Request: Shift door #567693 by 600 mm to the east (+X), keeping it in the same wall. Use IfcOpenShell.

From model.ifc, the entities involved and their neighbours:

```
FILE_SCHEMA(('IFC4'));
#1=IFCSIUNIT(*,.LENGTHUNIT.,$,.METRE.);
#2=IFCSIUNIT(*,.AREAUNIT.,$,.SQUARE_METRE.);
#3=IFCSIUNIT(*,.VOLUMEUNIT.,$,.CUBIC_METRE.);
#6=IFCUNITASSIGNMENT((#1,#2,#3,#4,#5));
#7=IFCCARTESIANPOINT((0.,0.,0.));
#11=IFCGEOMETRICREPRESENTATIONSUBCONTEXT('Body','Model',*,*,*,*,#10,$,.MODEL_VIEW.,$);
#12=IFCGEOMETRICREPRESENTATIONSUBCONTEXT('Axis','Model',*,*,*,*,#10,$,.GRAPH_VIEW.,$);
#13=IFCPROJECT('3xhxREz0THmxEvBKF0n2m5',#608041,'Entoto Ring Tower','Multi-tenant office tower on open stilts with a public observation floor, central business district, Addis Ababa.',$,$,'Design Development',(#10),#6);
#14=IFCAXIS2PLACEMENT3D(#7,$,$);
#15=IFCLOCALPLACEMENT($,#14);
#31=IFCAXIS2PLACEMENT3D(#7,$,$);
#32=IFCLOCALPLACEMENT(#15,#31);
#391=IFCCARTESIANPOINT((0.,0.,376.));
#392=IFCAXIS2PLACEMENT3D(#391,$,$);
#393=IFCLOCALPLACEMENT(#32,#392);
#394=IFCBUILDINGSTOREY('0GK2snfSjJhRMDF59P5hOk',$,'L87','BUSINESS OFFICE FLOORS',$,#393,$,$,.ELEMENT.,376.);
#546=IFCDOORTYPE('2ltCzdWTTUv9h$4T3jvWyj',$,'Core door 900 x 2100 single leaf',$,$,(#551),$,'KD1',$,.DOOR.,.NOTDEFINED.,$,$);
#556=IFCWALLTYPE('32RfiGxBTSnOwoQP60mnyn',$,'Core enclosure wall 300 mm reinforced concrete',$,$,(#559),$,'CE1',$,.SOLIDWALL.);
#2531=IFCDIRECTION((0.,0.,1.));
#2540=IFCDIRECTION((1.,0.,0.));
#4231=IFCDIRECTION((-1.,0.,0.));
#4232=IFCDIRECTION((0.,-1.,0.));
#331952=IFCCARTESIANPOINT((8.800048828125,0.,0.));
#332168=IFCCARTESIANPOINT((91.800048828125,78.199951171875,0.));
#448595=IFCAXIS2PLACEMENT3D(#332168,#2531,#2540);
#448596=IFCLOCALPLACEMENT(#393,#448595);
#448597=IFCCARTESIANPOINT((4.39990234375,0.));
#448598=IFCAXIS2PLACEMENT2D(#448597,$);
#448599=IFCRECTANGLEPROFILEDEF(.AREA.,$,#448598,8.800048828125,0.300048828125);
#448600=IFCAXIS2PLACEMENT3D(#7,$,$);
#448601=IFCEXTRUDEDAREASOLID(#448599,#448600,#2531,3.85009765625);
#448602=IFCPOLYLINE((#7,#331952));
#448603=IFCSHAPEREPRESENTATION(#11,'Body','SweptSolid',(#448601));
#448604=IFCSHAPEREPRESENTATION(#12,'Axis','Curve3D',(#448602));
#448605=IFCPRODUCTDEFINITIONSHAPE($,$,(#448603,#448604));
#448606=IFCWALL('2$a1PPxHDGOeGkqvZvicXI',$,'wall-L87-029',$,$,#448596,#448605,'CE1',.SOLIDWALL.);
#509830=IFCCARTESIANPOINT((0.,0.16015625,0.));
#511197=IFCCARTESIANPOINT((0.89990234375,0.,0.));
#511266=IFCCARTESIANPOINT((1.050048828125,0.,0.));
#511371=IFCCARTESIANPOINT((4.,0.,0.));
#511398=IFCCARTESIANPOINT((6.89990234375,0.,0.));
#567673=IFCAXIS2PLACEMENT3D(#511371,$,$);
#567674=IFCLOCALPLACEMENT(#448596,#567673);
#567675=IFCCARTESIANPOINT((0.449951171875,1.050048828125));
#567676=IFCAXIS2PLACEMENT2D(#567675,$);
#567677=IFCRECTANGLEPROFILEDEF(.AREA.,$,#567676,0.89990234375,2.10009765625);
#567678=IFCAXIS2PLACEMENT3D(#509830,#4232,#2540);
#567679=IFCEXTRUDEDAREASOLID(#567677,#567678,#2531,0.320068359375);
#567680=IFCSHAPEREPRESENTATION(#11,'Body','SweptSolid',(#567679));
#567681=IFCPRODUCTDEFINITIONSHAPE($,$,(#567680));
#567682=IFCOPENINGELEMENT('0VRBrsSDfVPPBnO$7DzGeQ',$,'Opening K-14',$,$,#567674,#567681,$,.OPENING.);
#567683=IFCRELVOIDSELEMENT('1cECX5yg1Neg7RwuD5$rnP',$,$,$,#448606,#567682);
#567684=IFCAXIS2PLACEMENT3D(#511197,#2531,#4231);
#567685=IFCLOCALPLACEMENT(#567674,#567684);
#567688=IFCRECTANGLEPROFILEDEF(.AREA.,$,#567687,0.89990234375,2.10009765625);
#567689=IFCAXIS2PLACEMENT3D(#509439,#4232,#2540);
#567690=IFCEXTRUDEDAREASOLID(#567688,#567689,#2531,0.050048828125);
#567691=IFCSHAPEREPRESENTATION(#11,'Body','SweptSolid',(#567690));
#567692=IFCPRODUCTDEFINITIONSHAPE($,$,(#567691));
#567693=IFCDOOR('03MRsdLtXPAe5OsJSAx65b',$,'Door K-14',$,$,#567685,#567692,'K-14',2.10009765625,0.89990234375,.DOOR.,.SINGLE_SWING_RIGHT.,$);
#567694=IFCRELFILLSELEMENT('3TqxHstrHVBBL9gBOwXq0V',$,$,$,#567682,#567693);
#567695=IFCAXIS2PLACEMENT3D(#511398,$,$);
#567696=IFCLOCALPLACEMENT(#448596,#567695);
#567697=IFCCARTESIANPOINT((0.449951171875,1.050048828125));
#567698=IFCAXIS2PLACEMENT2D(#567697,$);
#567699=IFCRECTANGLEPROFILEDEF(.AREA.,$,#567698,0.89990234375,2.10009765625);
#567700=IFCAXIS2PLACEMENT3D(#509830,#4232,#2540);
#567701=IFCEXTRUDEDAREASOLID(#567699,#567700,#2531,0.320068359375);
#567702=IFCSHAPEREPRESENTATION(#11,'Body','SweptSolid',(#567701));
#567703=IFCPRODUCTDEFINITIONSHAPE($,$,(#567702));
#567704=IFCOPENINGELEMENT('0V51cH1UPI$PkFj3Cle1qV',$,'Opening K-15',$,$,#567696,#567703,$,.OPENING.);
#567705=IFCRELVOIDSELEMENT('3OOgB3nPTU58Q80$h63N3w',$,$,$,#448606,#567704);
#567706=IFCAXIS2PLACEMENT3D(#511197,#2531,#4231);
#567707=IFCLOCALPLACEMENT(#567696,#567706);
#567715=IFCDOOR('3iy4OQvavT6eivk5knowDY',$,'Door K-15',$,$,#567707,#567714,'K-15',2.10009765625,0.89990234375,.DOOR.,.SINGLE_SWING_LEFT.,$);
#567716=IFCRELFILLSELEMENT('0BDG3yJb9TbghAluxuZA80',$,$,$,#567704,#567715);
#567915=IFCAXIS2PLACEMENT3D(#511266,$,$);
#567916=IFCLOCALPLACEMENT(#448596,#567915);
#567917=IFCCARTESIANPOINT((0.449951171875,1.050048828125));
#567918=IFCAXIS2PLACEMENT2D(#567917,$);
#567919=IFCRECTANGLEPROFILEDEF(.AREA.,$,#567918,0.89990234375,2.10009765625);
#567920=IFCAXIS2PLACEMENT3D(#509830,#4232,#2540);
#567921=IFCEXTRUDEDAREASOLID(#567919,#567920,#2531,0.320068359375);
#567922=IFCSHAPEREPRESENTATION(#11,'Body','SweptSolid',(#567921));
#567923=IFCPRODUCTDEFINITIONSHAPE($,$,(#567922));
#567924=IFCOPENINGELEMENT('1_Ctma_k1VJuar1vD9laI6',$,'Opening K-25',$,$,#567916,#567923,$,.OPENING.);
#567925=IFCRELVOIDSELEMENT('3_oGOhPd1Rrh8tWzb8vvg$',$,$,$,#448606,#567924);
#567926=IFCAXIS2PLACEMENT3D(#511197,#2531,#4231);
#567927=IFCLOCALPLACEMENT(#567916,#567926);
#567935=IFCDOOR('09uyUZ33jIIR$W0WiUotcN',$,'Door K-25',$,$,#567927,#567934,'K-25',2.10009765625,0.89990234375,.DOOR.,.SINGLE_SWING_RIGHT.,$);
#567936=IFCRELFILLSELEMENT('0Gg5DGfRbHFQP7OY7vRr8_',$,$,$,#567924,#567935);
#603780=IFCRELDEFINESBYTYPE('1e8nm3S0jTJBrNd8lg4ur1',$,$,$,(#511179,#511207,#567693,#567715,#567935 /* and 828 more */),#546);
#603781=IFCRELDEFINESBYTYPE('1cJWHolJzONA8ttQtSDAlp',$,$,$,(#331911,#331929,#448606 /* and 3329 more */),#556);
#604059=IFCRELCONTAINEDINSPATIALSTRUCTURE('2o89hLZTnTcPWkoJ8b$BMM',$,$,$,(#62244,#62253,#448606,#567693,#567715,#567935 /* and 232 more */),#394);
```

```python
import ifcopenshell
import ifcopenshell.api.geometry
import ifcopenshell.util.placement
import ifcopenshell.util.unit

model = ifcopenshell.open("model.ifc")
unit_scale = ifcopenshell.util.unit.calculate_unit_scale(model)

door = model.by_guid("03MRsdLtXPAe5OsJSAx65b")
opening = door.FillsVoids[0].RelatingOpeningElement
wall = opening.VoidsElements[0].RelatingBuildingElement

wall_matrix = ifcopenshell.util.placement.get_local_placement(wall.ObjectPlacement)
shift = wall_matrix[:3, 0] * 0.6 / unit_scale
before = ifcopenshell.util.placement.get_local_placement(door.ObjectPlacement)[:3, 3].copy()

# The door is placed relative to its opening, so it follows when the opening moves.
matrix = ifcopenshell.util.placement.get_local_placement(opening.ObjectPlacement)
matrix[:3, 3] += shift
ifcopenshell.api.geometry.edit_object_placement(
    model, product=opening, matrix=matrix, is_si=False, should_transform_children=True
)

after = ifcopenshell.util.placement.get_local_placement(door.ObjectPlacement)[:3, 3]
print("door moved by", (after - before).round(3) + 0.0)

model.write("model-out.ifc")
```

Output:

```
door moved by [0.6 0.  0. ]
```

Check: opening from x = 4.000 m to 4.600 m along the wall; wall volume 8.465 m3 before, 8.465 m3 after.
